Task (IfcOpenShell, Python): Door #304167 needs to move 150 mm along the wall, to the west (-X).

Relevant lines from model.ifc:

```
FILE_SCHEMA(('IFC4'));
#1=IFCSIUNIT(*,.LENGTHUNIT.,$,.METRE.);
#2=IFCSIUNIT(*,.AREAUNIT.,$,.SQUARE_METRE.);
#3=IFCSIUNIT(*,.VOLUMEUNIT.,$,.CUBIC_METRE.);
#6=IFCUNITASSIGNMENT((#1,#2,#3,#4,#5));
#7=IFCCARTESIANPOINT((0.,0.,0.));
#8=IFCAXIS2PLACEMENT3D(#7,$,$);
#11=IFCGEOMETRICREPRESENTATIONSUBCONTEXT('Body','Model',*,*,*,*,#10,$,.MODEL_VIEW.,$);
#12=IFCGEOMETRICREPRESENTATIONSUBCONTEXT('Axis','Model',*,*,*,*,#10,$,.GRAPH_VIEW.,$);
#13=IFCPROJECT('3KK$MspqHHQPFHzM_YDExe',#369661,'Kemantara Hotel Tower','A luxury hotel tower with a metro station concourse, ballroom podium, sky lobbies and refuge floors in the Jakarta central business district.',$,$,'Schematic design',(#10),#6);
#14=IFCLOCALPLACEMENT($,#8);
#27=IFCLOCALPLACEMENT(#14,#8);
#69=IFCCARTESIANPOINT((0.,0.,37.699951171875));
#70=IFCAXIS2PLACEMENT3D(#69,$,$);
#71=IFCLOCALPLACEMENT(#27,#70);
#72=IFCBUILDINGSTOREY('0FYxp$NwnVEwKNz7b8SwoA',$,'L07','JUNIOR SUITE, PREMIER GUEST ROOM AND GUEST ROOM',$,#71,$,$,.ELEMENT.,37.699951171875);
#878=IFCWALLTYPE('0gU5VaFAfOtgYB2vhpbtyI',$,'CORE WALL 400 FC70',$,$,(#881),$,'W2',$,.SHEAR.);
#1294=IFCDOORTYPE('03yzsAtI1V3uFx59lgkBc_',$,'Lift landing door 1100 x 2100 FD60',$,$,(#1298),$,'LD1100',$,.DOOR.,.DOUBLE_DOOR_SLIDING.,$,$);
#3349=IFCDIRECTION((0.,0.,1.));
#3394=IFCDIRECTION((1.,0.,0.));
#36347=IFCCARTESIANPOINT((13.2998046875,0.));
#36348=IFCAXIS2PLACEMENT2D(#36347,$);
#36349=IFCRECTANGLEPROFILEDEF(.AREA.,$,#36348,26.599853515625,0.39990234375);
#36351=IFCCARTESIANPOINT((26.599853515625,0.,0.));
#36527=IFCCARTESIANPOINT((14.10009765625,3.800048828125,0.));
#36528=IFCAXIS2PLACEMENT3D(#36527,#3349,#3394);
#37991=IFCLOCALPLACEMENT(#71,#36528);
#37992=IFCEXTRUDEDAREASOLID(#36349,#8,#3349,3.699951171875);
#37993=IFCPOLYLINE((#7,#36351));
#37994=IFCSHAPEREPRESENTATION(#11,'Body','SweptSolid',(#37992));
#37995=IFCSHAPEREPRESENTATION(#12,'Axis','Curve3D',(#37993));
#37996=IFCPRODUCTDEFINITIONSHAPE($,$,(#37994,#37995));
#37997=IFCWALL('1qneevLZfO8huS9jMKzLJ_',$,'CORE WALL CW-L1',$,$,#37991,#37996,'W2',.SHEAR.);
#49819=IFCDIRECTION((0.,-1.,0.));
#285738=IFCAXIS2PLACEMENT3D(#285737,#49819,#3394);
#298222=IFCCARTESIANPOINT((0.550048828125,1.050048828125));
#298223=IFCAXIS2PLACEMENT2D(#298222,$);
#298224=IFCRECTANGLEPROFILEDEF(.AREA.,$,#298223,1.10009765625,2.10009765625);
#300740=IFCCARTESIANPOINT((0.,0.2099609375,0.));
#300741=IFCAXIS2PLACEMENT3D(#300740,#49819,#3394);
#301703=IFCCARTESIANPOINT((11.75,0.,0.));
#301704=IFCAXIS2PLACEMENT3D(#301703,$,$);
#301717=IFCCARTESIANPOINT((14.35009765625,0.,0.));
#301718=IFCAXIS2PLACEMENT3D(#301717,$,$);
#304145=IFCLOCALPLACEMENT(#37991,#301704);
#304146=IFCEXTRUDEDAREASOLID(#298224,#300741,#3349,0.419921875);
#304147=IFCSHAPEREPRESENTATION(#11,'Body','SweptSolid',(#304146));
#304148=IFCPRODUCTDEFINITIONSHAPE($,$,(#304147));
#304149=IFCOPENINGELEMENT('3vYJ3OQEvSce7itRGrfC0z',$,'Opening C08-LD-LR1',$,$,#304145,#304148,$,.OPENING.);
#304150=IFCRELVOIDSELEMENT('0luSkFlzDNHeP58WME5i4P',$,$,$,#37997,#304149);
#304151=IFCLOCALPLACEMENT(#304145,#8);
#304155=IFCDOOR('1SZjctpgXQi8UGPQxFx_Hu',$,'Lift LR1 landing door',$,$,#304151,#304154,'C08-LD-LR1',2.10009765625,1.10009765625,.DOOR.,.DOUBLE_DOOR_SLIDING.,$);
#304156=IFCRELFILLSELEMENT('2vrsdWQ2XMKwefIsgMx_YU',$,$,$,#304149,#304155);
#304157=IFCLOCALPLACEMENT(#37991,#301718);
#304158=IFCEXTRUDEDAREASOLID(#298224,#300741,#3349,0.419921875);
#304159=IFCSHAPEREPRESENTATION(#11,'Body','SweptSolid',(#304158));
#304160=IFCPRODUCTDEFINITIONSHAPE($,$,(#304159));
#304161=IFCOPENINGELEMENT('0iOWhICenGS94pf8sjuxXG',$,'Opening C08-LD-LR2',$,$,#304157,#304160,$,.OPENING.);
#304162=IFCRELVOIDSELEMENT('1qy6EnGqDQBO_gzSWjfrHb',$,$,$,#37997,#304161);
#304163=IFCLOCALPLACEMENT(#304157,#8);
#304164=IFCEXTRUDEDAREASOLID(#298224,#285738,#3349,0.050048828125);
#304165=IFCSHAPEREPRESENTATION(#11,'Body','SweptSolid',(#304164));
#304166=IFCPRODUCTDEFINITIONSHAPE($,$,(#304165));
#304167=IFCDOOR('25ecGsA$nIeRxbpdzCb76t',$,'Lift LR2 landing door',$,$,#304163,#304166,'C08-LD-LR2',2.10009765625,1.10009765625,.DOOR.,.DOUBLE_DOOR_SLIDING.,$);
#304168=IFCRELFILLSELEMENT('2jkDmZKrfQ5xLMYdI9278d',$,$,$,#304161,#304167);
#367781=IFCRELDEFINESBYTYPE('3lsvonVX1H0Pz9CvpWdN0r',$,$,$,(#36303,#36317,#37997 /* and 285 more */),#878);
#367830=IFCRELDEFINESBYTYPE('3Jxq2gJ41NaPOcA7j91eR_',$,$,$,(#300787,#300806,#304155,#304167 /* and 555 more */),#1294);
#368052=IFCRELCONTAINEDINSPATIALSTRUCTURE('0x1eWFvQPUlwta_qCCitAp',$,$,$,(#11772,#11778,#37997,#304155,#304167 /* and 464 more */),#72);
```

```python
import ifcopenshell
import ifcopenshell.api.geometry
import ifcopenshell.util.placement
import ifcopenshell.util.unit

model = ifcopenshell.open("model.ifc")
unit_scale = ifcopenshell.util.unit.calculate_unit_scale(model)

door = model.by_guid("25ecGsA$nIeRxbpdzCb76t")
opening = door.FillsVoids[0].RelatingOpeningElement
wall = opening.VoidsElements[0].RelatingBuildingElement

wall_matrix = ifcopenshell.util.placement.get_local_placement(wall.ObjectPlacement)
shift = wall_matrix[:3, 0] * -0.15 / unit_scale
before = ifcopenshell.util.placement.get_local_placement(door.ObjectPlacement)[:3, 3].copy()

# The door is placed relative to its opening, so it follows when the opening moves.
matrix = ifcopenshell.util.placement.get_local_placement(opening.ObjectPlacement)
matrix[:3, 3] += shift
ifcopenshell.api.geometry.edit_object_placement(
    model, product=opening, matrix=matrix, is_si=False, should_transform_children=True
)

after = ifcopenshell.util.placement.get_local_placement(door.ObjectPlacement)[:3, 3]
print("door moved by", (after - before).round(3) + 0.0)

model.write("model_edited.ifc")
```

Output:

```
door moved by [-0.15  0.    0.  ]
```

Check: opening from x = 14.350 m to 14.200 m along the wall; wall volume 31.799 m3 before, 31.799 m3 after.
